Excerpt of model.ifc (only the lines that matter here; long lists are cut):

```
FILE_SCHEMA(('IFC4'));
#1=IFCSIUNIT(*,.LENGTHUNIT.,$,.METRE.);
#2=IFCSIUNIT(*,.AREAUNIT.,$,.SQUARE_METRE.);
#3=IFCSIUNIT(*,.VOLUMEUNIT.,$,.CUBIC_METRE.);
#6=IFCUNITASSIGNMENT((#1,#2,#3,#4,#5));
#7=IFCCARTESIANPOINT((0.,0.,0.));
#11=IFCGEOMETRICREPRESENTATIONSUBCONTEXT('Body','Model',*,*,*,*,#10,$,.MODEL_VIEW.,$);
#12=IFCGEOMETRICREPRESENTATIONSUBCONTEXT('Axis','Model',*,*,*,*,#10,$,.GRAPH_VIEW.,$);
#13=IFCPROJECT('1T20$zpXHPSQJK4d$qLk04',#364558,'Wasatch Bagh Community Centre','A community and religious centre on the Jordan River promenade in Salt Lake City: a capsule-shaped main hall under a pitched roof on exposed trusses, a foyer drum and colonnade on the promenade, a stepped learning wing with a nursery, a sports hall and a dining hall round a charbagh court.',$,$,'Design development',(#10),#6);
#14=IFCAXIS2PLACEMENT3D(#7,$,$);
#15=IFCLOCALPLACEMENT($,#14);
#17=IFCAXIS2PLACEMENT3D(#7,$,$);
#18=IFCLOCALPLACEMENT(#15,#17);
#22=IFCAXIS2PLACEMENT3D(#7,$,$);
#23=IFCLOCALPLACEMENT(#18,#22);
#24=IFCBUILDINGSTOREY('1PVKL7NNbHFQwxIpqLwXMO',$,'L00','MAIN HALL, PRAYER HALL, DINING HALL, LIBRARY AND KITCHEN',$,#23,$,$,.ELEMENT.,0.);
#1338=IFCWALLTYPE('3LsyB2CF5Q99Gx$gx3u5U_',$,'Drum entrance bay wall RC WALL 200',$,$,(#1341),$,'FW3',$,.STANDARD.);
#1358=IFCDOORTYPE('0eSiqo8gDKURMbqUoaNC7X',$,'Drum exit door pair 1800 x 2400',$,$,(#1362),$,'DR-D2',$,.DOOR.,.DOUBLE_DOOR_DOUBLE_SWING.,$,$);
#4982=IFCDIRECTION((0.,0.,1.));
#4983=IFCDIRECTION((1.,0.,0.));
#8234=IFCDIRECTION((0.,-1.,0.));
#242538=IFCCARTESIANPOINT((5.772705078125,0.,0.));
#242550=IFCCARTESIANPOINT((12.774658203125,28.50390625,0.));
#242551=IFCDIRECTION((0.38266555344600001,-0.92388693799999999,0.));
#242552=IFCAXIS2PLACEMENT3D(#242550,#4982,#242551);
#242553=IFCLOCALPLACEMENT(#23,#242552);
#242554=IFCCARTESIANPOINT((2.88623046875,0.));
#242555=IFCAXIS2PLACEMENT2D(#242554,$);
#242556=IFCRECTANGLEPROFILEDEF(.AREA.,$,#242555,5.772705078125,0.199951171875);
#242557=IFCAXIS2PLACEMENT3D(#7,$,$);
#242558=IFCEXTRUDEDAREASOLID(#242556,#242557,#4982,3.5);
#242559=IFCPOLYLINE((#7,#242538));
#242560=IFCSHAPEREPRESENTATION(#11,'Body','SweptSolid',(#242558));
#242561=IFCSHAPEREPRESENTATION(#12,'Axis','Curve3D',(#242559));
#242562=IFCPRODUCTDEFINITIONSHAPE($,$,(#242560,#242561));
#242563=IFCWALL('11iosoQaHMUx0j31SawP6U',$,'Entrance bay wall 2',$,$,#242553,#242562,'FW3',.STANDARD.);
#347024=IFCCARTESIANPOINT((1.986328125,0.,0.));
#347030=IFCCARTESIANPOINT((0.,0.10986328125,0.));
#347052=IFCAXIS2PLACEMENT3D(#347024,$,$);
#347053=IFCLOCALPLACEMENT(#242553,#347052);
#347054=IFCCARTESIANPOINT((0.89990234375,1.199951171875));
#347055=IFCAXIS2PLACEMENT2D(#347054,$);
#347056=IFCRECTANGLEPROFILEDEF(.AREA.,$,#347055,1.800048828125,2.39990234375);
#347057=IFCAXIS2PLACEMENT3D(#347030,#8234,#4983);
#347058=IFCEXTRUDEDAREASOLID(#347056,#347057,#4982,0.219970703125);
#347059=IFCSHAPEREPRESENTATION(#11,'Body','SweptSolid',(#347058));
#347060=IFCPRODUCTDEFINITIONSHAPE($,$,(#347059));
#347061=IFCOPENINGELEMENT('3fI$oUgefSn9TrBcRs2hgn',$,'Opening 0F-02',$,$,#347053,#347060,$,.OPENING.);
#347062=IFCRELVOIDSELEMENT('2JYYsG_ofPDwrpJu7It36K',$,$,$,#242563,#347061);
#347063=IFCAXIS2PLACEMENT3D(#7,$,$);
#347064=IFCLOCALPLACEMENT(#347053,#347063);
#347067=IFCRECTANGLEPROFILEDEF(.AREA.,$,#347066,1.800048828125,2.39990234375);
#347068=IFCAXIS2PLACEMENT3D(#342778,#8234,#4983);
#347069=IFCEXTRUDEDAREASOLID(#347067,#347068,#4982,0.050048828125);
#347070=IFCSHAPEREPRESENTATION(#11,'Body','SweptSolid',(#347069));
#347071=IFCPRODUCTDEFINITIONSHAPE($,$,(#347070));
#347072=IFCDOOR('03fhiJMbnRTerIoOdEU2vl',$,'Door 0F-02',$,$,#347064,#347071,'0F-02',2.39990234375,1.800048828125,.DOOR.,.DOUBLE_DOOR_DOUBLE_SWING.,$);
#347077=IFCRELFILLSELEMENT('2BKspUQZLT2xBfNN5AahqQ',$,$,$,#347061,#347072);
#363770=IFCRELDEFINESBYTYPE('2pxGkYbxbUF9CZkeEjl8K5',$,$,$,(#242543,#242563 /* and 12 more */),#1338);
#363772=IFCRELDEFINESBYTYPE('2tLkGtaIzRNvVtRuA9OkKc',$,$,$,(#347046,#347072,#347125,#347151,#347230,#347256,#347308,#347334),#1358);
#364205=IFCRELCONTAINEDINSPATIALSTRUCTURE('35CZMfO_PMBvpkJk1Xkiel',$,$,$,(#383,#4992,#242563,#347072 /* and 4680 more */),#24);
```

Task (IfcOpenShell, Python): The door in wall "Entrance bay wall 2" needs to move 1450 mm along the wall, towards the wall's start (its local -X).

```python
import ifcopenshell
import ifcopenshell.api.geometry
import ifcopenshell.util.placement
import ifcopenshell.util.unit

model = ifcopenshell.open("model.ifc")
unit_scale = ifcopenshell.util.unit.calculate_unit_scale(model)

door = model.by_id(347072)
opening = door.FillsVoids[0].RelatingOpeningElement
wall = opening.VoidsElements[0].RelatingBuildingElement

wall_matrix = ifcopenshell.util.placement.get_local_placement(wall.ObjectPlacement)
shift = wall_matrix[:3, 0] * -1.45 / unit_scale
before = ifcopenshell.util.placement.get_local_placement(door.ObjectPlacement)[:3, 3].copy()

# The door is placed relative to its opening, so it follows when the opening moves.
matrix = ifcopenshell.util.placement.get_local_placement(opening.ObjectPlacement)
matrix[:3, 3] += shift
ifcopenshell.api.geometry.edit_object_placement(
    model, product=opening, matrix=matrix, is_si=False, should_transform_children=True
)

after = ifcopenshell.util.placement.get_local_placement(door.ObjectPlacement)[:3, 3]
print("door moved by", (after - before).round(3) + 0.0)

model.write("model-out.ifc")
```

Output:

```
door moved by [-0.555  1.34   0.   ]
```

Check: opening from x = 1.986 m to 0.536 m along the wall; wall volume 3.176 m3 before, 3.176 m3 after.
